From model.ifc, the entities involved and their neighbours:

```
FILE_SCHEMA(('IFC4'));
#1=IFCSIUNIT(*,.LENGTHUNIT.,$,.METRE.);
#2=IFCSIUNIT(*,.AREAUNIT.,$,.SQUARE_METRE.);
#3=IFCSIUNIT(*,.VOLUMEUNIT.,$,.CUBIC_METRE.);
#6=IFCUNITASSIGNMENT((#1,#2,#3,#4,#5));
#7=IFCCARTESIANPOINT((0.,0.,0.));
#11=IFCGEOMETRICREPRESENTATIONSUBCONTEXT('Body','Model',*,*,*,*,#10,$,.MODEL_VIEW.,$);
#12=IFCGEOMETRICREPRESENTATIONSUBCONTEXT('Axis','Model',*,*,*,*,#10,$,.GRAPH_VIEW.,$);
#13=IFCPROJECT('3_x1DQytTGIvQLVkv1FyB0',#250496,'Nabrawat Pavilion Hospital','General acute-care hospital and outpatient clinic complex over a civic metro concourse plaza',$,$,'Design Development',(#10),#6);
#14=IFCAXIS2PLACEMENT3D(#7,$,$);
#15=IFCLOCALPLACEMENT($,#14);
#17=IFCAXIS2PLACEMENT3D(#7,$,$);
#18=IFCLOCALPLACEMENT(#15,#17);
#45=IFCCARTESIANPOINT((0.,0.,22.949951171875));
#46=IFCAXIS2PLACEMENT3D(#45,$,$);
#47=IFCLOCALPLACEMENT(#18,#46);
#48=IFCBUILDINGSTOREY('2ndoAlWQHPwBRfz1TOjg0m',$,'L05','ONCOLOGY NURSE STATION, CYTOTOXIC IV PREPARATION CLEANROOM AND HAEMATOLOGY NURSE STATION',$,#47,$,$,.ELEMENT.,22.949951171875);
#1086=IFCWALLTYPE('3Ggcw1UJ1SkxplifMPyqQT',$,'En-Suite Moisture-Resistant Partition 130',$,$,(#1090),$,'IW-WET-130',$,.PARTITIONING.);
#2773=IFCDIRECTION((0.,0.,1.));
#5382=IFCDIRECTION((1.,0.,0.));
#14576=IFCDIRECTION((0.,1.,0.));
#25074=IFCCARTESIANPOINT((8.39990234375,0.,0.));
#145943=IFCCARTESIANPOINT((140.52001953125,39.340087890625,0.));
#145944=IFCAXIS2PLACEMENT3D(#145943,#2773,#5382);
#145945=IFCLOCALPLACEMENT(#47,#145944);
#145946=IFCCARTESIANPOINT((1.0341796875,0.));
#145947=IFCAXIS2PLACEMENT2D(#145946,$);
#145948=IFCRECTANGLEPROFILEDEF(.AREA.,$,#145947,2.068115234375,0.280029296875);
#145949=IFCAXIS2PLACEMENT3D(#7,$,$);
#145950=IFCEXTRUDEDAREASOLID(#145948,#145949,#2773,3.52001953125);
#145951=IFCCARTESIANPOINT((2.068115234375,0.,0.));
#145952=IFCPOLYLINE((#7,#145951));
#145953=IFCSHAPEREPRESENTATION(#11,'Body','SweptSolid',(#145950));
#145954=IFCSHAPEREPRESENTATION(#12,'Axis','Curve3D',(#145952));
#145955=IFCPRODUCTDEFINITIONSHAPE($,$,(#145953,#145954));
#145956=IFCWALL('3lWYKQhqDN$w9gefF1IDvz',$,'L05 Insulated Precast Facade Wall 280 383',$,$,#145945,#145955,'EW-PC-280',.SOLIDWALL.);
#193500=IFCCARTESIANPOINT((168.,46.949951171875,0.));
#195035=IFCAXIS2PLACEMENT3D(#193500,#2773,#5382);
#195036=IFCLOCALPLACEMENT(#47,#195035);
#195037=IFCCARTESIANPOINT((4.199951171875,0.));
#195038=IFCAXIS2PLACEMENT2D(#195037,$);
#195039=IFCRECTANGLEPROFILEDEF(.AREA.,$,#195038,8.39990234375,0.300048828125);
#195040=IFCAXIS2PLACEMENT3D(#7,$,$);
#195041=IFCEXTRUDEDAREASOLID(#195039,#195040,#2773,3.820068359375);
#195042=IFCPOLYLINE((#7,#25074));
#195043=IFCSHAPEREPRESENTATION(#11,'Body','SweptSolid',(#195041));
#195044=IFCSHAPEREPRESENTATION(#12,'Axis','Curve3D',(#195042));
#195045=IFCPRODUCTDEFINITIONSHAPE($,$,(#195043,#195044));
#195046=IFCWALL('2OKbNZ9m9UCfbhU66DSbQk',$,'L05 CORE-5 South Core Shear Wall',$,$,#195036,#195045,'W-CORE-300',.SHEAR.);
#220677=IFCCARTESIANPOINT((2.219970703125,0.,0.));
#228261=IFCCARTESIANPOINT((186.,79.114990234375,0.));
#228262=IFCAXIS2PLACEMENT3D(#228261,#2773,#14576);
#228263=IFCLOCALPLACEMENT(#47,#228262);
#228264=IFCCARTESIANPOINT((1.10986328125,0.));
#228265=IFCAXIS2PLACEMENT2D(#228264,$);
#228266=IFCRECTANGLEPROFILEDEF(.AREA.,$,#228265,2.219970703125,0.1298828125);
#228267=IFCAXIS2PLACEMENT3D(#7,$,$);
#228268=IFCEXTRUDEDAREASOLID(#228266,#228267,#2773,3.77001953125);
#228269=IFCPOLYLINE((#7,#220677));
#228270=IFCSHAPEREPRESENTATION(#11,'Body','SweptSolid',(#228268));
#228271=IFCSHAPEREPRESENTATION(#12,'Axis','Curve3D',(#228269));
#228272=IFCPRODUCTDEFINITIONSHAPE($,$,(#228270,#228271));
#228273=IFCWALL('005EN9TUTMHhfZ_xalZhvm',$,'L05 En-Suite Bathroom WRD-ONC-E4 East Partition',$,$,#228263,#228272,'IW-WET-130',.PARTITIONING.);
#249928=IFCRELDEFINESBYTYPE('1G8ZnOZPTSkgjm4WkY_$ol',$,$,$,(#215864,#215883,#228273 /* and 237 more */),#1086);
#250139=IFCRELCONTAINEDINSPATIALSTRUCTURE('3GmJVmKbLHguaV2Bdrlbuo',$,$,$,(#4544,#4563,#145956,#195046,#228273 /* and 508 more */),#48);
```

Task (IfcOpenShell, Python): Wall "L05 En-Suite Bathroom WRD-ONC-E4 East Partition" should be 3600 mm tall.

```python
import ifcopenshell
import ifcopenshell.geom
import ifcopenshell.util.representation
import ifcopenshell.util.shape

model = ifcopenshell.open("model.ifc")
settings = ifcopenshell.geom.settings()


def volume(element):
    """Net volume in cubic metres, openings subtracted."""
    shape = ifcopenshell.geom.create_shape(settings, element)
    return ifcopenshell.util.shape.get_volume(shape.geometry)


wall = model.by_guid("005EN9TUTMHhfZ_xalZhvm")
before = volume(wall)

body = ifcopenshell.util.representation.get_representation(wall, "Model", "Body")
solid = body.Items[0]
old_height = solid.Depth
solid.Depth = 3.6
after = volume(wall)

print(f"height {old_height:g} -> {solid.Depth:g}, volume {before:.3f} -> {after:.3f} m3")

model.write("model_v2.ifc")
```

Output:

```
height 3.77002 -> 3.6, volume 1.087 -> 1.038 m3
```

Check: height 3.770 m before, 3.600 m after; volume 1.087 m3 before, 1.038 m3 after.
